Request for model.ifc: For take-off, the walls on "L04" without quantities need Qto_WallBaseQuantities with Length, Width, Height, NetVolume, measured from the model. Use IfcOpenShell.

First a look at what the model holds.

```python
import ifcopenshell
import ifcopenshell.util.element
import ifcopenshell.util.unit

model = ifcopenshell.open("model.ifc")
print(model.schema)
for unit_type in ("LENGTHUNIT", "AREAUNIT", "VOLUMEUNIT"):
    print(unit_type, ifcopenshell.util.unit.calculate_unit_scale(model, unit_type))
storey = next(s for s in model.by_type("IfcBuildingStorey") if s.Name == "L04")
walls = [e for e in ifcopenshell.util.element.get_decomposition(storey) if e.is_a("IfcWall")]
for e in sorted(walls, key=lambda e: e.id()):
    print(e.id(), e.is_a(), e.Name, list(ifcopenshell.util.element.get_psets(e, qtos_only=True)), sep=" | ")
```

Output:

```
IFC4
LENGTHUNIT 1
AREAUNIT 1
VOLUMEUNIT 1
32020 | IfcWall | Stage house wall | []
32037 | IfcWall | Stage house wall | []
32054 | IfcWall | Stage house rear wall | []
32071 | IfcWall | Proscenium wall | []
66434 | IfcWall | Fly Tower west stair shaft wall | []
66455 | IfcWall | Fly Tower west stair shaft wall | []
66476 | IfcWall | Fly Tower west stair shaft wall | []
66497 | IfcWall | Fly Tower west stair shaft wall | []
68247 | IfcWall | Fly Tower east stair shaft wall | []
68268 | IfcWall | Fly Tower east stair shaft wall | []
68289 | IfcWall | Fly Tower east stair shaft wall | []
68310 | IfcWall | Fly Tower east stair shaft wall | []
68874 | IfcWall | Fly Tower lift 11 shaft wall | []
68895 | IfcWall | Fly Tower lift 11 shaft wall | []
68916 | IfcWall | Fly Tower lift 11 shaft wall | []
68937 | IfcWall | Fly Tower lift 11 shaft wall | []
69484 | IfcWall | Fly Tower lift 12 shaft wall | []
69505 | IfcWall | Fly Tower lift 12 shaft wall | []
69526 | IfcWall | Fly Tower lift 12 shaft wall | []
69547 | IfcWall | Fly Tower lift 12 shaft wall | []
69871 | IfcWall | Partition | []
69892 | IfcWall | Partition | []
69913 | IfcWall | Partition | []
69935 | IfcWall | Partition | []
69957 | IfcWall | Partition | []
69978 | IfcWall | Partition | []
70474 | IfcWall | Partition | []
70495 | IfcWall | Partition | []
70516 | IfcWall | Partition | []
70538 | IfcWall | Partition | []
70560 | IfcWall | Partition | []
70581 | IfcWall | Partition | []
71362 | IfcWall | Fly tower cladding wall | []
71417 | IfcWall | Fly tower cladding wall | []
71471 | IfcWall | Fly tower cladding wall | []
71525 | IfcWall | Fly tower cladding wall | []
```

```python
import ifcopenshell
import ifcopenshell.api.pset
import ifcopenshell.geom
import ifcopenshell.util.element
import ifcopenshell.util.shape
import ifcopenshell.util.unit

model = ifcopenshell.open("model.ifc")
unit_scale = ifcopenshell.util.unit.calculate_unit_scale(model)
volume_scale = ifcopenshell.util.unit.calculate_unit_scale(model, "VOLUMEUNIT")
settings = ifcopenshell.geom.settings()

storey = next(s for s in model.by_type("IfcBuildingStorey") if s.Name == "L04")
walls = [e for e in ifcopenshell.util.element.get_decomposition(storey) if e.is_a("IfcWall")]

for e in sorted(walls, key=lambda e: e.id()):
    if ifcopenshell.util.element.get_psets(e, qtos_only=True, should_inherit=False):
        continue
    # Geometry comes back in metres, in the element's own axes.
    shape = ifcopenshell.geom.create_shape(settings, e)
    values = {
        "Length": ifcopenshell.util.shape.get_x(shape.geometry) / unit_scale,
        "Width": ifcopenshell.util.shape.get_y(shape.geometry) / unit_scale,
        "Height": ifcopenshell.util.shape.get_z(shape.geometry) / unit_scale,
        "NetVolume": ifcopenshell.util.shape.get_volume(shape.geometry) / volume_scale,
    }
    qto = ifcopenshell.api.pset.add_qto(model, product=e, name="Qto_WallBaseQuantities")
    ifcopenshell.api.pset.edit_qto(model, qto=qto, properties=values)
    print(e.id(), {k: round(v, 3) for k, v in values.items()})

model.write("model-out.ifc")
```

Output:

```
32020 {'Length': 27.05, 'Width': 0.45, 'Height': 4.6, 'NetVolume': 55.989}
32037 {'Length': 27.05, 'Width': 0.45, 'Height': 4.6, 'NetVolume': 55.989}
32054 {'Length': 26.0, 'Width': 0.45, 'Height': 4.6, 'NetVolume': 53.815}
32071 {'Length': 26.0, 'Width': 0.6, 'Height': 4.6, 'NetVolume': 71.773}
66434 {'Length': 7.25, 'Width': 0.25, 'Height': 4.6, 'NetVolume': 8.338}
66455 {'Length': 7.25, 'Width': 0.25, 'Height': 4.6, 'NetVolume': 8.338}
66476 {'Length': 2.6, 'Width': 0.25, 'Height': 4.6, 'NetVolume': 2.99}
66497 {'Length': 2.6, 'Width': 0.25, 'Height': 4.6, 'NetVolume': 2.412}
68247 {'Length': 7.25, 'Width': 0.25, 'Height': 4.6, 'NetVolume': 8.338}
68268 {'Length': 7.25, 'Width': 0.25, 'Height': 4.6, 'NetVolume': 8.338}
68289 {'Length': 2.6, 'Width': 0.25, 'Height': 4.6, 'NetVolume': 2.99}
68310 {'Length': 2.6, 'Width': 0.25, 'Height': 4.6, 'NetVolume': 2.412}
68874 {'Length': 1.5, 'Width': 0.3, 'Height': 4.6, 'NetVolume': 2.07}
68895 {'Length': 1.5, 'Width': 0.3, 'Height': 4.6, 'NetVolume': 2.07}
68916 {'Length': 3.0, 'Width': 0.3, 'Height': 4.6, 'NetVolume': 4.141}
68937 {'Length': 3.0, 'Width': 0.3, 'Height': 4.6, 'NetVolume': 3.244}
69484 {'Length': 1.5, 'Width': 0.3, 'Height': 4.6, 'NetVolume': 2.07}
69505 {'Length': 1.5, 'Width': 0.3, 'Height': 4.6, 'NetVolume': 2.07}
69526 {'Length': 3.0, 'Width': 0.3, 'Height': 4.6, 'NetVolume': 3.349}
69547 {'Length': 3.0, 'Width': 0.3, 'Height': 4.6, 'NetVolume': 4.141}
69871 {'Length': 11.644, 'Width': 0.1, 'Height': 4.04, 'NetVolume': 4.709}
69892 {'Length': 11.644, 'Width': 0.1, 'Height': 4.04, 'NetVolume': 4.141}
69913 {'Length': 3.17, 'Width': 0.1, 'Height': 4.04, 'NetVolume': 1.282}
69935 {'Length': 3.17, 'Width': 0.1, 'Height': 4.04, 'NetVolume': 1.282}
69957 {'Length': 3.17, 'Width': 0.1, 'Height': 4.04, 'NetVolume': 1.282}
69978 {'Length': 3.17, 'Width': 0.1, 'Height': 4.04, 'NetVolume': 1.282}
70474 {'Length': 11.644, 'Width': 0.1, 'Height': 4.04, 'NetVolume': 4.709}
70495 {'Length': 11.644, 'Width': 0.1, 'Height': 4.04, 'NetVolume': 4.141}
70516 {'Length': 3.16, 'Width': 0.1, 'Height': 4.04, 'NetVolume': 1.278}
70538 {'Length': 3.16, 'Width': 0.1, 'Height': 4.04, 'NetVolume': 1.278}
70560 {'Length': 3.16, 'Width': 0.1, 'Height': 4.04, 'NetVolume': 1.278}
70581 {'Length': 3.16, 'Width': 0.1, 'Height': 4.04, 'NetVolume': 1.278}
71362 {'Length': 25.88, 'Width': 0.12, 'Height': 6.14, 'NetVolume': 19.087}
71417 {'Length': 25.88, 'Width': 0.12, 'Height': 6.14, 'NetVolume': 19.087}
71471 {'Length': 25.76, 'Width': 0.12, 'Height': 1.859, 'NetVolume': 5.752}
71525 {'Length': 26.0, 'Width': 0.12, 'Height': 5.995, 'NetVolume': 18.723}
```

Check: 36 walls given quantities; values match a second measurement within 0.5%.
